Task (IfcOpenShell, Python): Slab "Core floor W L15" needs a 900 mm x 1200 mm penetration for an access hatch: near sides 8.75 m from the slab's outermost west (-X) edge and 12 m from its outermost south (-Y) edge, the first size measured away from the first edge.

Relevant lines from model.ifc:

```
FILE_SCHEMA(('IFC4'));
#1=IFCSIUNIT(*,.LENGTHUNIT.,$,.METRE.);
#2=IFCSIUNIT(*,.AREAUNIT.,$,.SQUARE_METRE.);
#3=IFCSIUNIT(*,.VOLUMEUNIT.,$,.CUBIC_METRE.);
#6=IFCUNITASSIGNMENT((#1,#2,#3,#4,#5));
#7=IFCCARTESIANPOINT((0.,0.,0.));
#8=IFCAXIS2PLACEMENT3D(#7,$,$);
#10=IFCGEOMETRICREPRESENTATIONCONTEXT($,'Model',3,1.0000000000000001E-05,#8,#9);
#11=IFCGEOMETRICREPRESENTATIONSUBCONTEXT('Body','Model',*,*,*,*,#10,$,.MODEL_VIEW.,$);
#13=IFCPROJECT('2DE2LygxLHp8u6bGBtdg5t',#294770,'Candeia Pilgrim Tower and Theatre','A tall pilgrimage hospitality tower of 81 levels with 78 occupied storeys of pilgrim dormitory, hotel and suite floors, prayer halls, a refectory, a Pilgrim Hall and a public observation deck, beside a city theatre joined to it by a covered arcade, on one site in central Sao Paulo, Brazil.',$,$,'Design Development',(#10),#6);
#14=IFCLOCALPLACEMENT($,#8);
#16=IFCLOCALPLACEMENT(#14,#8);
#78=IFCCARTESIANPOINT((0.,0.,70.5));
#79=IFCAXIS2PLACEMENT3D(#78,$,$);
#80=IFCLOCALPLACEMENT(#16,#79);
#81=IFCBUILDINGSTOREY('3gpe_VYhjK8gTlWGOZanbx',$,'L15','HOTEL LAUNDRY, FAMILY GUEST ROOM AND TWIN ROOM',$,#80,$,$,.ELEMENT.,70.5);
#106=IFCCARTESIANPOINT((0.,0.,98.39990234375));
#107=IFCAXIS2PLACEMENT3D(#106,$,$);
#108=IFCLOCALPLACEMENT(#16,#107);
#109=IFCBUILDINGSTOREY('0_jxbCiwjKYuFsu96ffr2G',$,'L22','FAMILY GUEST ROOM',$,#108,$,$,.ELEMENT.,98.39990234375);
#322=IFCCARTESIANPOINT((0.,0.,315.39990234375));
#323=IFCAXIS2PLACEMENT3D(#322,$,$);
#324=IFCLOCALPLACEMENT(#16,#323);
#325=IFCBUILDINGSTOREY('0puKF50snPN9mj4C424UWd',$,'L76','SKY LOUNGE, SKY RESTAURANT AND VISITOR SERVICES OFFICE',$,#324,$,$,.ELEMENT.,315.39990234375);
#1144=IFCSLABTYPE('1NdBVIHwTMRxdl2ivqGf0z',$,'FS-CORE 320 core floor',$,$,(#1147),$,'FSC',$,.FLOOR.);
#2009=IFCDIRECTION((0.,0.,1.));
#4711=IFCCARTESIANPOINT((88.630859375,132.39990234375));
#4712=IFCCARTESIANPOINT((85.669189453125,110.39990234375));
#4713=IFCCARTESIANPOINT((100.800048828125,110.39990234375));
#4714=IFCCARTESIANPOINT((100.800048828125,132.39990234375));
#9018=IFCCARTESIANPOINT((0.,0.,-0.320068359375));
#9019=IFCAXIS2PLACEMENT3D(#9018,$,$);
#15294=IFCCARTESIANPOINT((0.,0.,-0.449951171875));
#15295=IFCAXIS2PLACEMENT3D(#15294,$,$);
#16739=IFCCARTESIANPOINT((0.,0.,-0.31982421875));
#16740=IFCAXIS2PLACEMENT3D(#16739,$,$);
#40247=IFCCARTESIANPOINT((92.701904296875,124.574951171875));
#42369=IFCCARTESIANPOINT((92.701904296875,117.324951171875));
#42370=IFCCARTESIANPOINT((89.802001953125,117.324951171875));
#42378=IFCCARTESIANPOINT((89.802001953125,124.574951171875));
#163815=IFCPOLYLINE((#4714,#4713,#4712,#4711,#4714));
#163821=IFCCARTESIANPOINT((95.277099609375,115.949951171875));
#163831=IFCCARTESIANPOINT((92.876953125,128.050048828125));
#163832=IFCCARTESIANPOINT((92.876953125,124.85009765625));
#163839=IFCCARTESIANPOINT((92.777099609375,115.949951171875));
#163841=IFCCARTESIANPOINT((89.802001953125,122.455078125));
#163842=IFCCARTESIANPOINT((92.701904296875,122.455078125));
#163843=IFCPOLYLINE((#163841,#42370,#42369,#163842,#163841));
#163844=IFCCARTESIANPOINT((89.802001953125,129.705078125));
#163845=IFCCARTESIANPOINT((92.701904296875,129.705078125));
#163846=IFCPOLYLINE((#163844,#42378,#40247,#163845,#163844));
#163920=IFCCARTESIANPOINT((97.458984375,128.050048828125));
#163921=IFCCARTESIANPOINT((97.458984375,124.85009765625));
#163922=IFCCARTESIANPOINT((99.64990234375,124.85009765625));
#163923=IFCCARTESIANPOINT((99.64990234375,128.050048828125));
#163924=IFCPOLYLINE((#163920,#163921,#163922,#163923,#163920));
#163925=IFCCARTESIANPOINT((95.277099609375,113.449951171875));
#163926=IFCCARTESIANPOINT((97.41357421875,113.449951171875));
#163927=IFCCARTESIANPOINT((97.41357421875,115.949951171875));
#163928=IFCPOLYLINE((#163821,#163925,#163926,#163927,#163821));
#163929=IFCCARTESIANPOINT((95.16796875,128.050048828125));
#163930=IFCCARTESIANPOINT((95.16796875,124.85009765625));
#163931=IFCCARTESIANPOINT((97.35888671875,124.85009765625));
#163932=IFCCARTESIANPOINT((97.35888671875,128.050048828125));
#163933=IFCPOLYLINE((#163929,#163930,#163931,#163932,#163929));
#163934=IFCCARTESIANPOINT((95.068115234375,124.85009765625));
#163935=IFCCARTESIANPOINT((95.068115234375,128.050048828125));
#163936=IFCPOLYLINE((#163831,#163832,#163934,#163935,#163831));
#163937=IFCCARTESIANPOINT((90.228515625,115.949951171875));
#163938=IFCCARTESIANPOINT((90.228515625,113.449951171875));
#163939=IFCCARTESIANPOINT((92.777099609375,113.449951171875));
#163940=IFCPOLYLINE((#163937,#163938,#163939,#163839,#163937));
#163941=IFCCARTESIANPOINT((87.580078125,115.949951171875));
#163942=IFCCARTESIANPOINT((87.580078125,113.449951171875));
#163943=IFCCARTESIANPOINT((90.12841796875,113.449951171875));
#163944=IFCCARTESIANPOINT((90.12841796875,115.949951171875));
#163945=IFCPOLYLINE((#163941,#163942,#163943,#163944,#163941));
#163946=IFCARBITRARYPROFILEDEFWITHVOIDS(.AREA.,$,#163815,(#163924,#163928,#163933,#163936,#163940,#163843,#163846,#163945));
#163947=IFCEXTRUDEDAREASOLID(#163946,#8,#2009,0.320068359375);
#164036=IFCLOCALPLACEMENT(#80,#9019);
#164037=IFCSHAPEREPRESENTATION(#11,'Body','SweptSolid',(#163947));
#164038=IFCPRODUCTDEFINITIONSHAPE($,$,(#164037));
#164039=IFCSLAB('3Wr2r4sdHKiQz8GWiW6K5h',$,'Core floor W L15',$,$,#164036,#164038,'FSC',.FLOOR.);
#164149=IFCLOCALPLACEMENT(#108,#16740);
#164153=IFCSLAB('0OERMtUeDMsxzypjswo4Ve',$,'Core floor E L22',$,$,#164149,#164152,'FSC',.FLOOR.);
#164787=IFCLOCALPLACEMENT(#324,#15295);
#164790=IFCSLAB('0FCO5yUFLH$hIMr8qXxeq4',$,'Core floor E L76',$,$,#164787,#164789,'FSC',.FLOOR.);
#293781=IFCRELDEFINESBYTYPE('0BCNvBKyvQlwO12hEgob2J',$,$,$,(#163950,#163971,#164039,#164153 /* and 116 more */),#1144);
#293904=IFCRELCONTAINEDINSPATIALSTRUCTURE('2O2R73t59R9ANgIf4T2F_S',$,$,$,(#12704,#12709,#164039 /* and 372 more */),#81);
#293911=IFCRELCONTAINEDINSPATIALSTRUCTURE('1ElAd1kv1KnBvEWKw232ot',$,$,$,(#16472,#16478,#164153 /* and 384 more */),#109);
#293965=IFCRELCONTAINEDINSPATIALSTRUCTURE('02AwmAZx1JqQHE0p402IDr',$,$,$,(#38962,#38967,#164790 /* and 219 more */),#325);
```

```python
import numpy as np
import ifcopenshell
import ifcopenshell.api.feature
import ifcopenshell.api.geometry
import ifcopenshell.api.root
import ifcopenshell.geom
import ifcopenshell.util.placement
import ifcopenshell.util.representation
import ifcopenshell.util.shape
import ifcopenshell.util.unit

model = ifcopenshell.open("model.ifc")
unit_scale = ifcopenshell.util.unit.calculate_unit_scale(model)
settings = ifcopenshell.geom.settings()


def volume(element):
    """Net volume in cubic metres, openings subtracted."""
    shape = ifcopenshell.geom.create_shape(settings, element)
    return ifcopenshell.util.shape.get_volume(shape.geometry)


slab = model.by_guid("3Wr2r4sdHKiQz8GWiW6K5h")
before = volume(slab)

# Extent in the slab's own axes, in metres. The edges named are its -X and -Y sides.
slab_shape = ifcopenshell.geom.create_shape(settings, slab)
vertices = ifcopenshell.util.shape.get_vertices(slab_shape.geometry)
x_min, y_min, bottom = vertices.min(axis=0)
top = vertices[:, 2].max()

opening = ifcopenshell.api.root.create_entity(model, ifc_class="IfcOpeningElement", name="Access hatch opening", predefined_type="OPENING")
context = ifcopenshell.util.representation.get_context(model, "Model", "Body", "MODEL_VIEW")
width, depth = 0.9, 1.2
outline = [(0.0, 0.0), (width, 0.0), (width, depth), (0.0, depth), (0.0, 0.0)]
# Overshoot both faces by 50 mm so the cut is clean.
shape = ifcopenshell.api.geometry.add_slab_representation(
    model, context=context, depth=top - bottom + 0.1, polyline=outline
)
ifcopenshell.api.geometry.assign_representation(model, product=opening, representation=shape)

matrix = ifcopenshell.util.placement.get_local_placement(slab.ObjectPlacement)
matrix[:, 3] = matrix @ np.append(np.array([x_min + 8.75, y_min + 12, bottom - 0.05]) / unit_scale, 1.0)
ifcopenshell.api.geometry.edit_object_placement(model, product=opening, matrix=matrix, is_si=False)
ifcopenshell.api.feature.add_feature(model, feature=opening, element=slab)

after = volume(slab)

print(f"slab volume {before:.3f} -> {after:.3f} m3")

model.write("model_v2.ifc")
```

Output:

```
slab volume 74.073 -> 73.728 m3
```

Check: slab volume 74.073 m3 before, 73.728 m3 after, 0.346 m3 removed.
